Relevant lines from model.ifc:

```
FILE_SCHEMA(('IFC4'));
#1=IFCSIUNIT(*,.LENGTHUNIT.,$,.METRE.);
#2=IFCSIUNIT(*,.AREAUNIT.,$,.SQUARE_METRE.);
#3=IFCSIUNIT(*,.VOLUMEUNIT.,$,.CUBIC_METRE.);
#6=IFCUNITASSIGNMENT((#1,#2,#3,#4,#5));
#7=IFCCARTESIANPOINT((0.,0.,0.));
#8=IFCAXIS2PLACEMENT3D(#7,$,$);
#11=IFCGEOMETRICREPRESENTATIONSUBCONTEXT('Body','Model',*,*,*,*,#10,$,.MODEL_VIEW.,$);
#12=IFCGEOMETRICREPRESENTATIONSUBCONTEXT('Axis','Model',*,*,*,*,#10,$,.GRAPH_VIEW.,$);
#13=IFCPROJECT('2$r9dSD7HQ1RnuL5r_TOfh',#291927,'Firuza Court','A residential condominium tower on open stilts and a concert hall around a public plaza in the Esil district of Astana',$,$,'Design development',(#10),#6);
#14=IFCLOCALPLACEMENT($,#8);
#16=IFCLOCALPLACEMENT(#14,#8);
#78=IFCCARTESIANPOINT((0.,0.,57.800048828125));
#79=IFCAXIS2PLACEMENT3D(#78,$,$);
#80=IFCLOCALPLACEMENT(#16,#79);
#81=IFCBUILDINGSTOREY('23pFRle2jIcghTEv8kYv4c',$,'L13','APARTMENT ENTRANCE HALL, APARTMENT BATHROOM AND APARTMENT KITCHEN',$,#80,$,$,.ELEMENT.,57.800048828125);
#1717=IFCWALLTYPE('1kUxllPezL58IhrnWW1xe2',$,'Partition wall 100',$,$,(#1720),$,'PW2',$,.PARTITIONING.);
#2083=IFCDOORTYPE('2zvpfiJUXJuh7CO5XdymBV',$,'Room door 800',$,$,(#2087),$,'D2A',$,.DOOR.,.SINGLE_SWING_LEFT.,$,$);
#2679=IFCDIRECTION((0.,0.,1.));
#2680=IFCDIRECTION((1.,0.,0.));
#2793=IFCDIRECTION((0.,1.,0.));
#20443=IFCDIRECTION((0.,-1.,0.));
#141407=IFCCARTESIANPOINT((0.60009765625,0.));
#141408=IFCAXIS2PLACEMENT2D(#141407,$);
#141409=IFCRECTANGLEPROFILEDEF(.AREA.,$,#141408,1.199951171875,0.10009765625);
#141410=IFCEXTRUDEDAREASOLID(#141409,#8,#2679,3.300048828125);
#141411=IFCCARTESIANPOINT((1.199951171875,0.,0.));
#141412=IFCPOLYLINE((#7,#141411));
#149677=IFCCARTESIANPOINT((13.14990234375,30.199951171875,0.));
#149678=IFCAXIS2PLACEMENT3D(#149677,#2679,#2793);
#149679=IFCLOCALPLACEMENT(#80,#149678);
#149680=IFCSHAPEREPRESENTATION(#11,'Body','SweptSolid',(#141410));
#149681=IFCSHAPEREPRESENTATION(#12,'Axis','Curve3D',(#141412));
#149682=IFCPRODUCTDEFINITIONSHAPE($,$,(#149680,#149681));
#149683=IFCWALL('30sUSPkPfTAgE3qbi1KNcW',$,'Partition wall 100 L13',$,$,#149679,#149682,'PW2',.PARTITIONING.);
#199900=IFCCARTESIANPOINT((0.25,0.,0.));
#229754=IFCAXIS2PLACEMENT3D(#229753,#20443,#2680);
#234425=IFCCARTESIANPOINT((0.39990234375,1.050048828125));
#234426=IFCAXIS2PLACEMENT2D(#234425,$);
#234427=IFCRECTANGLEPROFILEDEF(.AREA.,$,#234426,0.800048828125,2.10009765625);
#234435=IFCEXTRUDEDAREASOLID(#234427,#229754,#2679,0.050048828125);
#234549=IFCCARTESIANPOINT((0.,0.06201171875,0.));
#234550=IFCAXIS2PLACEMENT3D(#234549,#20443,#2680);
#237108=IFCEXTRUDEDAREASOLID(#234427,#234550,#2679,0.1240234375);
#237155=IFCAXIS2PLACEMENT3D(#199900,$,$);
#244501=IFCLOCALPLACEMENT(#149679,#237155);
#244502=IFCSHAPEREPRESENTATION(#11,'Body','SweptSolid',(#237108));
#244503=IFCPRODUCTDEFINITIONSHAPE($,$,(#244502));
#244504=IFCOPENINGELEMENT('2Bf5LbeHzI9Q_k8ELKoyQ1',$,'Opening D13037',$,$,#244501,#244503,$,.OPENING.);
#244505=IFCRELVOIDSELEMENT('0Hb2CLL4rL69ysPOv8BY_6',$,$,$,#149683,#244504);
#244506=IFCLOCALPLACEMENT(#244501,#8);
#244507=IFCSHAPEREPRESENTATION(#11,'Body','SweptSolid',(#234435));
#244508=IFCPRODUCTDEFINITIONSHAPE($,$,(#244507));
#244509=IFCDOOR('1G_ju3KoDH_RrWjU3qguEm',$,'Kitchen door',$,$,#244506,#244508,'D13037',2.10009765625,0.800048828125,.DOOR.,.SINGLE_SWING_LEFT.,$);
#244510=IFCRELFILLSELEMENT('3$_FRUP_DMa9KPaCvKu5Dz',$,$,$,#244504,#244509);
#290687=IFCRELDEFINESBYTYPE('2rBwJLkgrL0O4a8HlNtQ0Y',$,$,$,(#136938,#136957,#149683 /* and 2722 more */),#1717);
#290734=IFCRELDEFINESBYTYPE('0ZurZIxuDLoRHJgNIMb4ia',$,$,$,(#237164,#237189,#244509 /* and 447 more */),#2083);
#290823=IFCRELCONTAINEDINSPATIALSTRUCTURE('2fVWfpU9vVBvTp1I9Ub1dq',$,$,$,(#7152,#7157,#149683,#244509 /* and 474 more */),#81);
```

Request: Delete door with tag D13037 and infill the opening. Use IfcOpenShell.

```python
import ifcopenshell
import ifcopenshell.api.feature
import ifcopenshell.api.root
import ifcopenshell.geom
import ifcopenshell.util.shape

model = ifcopenshell.open("model.ifc")
settings = ifcopenshell.geom.settings()


def volume(element):
    """Net volume in cubic metres, openings subtracted."""
    shape = ifcopenshell.geom.create_shape(settings, element)
    return ifcopenshell.util.shape.get_volume(shape.geometry)


door = model.by_id(244509)
opening = door.FillsVoids[0].RelatingOpeningElement
wall = opening.VoidsElements[0].RelatingBuildingElement
before = volume(wall)

ifcopenshell.api.root.remove_product(model, product=door)
ifcopenshell.api.feature.remove_feature(model, feature=opening)

after = volume(wall)

print(f"wall volume {before:.3f} -> {after:.3f} m3")

model.write("model_v2.ifc")
```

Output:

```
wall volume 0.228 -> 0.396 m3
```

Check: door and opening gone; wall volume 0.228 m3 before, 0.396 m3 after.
